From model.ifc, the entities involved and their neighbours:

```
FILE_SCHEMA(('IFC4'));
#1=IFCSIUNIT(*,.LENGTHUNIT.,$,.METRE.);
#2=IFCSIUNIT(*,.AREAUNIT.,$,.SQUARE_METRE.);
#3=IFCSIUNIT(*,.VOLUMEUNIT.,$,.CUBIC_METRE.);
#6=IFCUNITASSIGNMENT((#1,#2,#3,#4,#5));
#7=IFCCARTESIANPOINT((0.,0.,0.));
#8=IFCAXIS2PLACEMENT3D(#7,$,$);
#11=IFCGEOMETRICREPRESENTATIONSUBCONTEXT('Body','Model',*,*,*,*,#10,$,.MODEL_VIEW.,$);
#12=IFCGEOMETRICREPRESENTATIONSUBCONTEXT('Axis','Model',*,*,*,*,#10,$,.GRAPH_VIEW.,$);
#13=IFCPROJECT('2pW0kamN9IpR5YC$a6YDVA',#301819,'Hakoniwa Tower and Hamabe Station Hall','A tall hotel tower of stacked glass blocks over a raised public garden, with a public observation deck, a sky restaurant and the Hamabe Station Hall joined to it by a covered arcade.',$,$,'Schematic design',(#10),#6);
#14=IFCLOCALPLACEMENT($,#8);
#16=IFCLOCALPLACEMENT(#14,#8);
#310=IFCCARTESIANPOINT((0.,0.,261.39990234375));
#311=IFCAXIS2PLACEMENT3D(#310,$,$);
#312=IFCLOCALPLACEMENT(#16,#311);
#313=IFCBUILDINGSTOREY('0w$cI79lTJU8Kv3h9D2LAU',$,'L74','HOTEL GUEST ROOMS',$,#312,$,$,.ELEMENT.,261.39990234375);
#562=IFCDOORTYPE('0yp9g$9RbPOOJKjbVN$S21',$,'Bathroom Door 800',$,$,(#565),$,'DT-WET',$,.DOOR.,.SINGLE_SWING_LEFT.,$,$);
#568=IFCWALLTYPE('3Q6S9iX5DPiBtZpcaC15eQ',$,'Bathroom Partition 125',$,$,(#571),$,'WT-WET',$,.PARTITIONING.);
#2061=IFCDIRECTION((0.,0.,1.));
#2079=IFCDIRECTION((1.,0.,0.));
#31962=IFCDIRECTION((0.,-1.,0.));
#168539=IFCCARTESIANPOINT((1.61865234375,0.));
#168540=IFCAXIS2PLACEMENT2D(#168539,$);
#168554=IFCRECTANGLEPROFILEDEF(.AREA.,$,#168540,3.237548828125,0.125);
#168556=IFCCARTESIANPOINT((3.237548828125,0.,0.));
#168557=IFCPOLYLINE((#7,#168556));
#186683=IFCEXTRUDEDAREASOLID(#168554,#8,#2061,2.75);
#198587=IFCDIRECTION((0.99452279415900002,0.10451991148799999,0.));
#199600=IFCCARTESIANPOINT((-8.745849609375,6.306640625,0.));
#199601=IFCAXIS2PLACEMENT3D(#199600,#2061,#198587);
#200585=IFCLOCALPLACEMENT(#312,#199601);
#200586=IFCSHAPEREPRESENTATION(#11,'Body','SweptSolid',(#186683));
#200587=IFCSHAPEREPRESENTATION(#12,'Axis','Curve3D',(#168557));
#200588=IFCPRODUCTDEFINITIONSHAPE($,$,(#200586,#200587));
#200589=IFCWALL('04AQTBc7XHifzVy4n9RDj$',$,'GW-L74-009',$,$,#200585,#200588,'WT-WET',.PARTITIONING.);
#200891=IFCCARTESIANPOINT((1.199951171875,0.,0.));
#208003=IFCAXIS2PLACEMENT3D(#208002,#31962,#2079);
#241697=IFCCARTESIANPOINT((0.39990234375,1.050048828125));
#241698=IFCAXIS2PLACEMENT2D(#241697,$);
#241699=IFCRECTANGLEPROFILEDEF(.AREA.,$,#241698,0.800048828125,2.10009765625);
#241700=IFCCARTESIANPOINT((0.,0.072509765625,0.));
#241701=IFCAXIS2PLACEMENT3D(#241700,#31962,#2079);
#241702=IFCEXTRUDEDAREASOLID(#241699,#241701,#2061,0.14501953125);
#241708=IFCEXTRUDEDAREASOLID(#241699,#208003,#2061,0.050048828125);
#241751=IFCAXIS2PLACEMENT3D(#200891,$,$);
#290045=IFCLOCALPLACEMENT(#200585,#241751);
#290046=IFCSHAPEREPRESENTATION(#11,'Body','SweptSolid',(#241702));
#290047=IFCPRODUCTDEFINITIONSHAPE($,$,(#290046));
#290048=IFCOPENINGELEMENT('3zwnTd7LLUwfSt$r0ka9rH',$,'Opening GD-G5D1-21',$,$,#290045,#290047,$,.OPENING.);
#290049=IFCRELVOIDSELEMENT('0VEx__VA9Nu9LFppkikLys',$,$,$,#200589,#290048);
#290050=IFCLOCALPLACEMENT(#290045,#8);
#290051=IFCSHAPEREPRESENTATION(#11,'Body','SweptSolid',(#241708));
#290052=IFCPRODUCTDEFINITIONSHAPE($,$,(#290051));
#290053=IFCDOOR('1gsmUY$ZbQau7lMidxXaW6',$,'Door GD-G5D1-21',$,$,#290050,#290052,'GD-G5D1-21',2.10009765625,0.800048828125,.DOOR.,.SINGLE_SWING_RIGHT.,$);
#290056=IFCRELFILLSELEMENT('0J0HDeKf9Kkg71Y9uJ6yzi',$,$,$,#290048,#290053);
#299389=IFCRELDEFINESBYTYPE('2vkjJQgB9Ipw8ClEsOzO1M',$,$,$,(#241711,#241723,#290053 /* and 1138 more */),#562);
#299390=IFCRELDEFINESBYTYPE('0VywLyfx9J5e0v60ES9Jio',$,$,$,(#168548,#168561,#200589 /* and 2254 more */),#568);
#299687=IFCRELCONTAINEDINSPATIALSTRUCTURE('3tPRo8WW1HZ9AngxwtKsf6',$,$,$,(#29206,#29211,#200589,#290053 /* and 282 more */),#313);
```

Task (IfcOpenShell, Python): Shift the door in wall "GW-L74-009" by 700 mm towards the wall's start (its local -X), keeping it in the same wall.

```python
import ifcopenshell
import ifcopenshell.api.geometry
import ifcopenshell.util.placement
import ifcopenshell.util.unit

model = ifcopenshell.open("model.ifc")
unit_scale = ifcopenshell.util.unit.calculate_unit_scale(model)

door = model.by_id(290053)
opening = door.FillsVoids[0].RelatingOpeningElement
wall = opening.VoidsElements[0].RelatingBuildingElement

wall_matrix = ifcopenshell.util.placement.get_local_placement(wall.ObjectPlacement)
shift = wall_matrix[:3, 0] * -0.7 / unit_scale
before = ifcopenshell.util.placement.get_local_placement(door.ObjectPlacement)[:3, 3].copy()

# The door is placed relative to its opening, so it follows when the opening moves.
matrix = ifcopenshell.util.placement.get_local_placement(opening.ObjectPlacement)
matrix[:3, 3] += shift
ifcopenshell.api.geometry.edit_object_placement(
    model, product=opening, matrix=matrix, is_si=False, should_transform_children=True
)

after = ifcopenshell.util.placement.get_local_placement(door.ObjectPlacement)[:3, 3]
print("door moved by", (after - before).round(3) + 0.0)

model.write("model_v2.ifc")
```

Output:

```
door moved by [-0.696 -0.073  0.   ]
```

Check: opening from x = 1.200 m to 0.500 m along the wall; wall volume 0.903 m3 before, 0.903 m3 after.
